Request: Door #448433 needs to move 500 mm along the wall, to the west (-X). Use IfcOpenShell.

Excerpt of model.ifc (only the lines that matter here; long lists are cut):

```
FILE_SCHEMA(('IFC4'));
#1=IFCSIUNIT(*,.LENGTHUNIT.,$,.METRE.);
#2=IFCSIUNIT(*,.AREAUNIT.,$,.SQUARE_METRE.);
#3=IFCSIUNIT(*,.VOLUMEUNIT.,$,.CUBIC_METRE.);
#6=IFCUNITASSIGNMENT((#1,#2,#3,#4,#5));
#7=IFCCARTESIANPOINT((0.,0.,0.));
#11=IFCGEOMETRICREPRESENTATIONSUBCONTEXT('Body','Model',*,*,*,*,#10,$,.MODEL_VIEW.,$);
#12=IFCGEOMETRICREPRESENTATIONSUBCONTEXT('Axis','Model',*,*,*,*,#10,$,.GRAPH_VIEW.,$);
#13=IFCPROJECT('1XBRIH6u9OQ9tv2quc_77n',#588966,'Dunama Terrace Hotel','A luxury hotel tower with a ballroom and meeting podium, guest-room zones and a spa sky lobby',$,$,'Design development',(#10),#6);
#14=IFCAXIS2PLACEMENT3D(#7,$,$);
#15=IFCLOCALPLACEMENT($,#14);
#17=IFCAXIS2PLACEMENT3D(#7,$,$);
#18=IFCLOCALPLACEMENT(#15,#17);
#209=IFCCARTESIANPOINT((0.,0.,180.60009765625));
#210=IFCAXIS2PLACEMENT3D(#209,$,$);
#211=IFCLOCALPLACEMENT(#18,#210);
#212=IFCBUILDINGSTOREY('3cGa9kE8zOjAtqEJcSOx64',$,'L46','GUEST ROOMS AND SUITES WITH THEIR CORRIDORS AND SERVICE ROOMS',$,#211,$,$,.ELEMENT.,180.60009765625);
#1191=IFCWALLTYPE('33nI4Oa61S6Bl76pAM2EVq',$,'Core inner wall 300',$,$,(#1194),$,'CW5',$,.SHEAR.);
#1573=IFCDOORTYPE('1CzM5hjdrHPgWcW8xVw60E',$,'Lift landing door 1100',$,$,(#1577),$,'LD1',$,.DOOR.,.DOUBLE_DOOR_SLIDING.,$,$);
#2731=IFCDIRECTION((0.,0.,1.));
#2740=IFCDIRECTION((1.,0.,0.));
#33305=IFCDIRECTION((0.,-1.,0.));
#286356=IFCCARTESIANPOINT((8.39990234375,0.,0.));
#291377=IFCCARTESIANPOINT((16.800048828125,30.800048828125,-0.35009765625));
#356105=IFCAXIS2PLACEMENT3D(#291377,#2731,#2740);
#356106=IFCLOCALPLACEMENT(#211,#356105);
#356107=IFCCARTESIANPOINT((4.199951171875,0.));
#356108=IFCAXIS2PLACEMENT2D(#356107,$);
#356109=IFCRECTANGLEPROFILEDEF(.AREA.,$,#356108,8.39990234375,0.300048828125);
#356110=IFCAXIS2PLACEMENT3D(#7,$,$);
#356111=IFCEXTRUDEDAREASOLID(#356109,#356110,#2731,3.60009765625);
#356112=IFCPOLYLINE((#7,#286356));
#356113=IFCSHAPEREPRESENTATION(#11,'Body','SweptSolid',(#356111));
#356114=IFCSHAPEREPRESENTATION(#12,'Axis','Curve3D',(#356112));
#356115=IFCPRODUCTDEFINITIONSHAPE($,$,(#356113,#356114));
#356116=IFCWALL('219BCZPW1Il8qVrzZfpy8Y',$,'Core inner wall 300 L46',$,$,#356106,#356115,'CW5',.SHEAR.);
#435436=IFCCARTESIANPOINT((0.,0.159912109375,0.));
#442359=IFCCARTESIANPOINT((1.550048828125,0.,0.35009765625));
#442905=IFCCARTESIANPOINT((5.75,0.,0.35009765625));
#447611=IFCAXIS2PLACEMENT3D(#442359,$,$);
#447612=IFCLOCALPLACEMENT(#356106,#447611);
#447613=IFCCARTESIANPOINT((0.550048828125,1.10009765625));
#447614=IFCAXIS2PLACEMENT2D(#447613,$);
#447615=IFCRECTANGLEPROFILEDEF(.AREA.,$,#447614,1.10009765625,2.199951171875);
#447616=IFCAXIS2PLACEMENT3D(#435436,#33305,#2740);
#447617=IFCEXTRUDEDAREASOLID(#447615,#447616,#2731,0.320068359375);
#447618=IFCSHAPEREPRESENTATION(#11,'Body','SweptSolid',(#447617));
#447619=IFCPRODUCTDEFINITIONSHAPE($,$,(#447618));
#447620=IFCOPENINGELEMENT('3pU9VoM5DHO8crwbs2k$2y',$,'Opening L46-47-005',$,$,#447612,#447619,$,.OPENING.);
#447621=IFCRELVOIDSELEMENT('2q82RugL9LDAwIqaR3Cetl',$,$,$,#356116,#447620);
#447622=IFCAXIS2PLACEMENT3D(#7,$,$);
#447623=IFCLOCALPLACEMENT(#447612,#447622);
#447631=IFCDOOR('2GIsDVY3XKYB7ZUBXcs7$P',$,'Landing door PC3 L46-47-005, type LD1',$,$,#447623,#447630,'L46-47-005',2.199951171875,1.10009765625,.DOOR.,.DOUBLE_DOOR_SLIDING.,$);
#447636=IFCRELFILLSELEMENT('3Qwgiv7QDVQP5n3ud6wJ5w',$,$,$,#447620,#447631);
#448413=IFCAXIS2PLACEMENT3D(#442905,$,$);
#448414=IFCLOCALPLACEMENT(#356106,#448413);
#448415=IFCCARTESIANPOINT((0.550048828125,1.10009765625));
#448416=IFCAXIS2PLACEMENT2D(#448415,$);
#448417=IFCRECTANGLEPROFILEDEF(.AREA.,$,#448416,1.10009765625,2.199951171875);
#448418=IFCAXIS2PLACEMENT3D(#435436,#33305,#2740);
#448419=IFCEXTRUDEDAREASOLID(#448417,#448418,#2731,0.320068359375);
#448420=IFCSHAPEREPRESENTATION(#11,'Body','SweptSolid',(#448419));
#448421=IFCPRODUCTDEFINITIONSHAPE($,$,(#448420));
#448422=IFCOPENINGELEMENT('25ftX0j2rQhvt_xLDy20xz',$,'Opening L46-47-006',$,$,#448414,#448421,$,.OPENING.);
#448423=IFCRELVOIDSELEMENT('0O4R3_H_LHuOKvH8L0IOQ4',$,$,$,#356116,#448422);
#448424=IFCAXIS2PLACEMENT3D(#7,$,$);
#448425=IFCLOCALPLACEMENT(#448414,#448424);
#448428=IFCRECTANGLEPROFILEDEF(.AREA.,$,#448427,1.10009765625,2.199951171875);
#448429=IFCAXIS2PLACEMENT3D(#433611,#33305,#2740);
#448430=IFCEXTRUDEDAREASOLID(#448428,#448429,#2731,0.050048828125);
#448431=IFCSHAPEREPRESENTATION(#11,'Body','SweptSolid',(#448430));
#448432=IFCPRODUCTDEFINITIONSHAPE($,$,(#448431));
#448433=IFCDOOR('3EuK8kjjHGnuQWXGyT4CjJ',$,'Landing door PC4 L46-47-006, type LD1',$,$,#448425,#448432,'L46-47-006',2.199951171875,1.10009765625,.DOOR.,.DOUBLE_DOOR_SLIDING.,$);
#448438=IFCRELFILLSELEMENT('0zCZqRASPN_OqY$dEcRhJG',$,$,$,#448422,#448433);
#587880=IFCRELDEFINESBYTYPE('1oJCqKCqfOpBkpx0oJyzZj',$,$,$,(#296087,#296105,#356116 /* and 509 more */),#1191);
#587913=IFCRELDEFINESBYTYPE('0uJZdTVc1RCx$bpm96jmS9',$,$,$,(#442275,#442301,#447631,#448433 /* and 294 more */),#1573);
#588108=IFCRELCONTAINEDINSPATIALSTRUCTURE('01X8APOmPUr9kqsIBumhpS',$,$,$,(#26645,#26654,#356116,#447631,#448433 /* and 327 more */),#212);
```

```python
import ifcopenshell
import ifcopenshell.api.geometry
import ifcopenshell.util.placement

model = ifcopenshell.open("model.ifc")

door = model.by_guid("3EuK8kjjHGnuQWXGyT4CjJ")
opening = door.FillsVoids[0].RelatingOpeningElement
wall = opening.VoidsElements[0].RelatingBuildingElement

wall_matrix = ifcopenshell.util.placement.get_local_placement(wall.ObjectPlacement)
shift = wall_matrix[:3, 0] * -0.5
before = ifcopenshell.util.placement.get_local_placement(door.ObjectPlacement)[:3, 3].copy()

# The door is placed relative to its opening, so it follows when the opening moves.
matrix = ifcopenshell.util.placement.get_local_placement(opening.ObjectPlacement)
matrix[:3, 3] += shift
ifcopenshell.api.geometry.edit_object_placement(
    model, product=opening, matrix=matrix, is_si=False, should_transform_children=True
)

after = ifcopenshell.util.placement.get_local_placement(door.ObjectPlacement)[:3, 3]
print("door moved by", (after - before).round(3) + 0.0)

model.write("model_rev.ifc")
```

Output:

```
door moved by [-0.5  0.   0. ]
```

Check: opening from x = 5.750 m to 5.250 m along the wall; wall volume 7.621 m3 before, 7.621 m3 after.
